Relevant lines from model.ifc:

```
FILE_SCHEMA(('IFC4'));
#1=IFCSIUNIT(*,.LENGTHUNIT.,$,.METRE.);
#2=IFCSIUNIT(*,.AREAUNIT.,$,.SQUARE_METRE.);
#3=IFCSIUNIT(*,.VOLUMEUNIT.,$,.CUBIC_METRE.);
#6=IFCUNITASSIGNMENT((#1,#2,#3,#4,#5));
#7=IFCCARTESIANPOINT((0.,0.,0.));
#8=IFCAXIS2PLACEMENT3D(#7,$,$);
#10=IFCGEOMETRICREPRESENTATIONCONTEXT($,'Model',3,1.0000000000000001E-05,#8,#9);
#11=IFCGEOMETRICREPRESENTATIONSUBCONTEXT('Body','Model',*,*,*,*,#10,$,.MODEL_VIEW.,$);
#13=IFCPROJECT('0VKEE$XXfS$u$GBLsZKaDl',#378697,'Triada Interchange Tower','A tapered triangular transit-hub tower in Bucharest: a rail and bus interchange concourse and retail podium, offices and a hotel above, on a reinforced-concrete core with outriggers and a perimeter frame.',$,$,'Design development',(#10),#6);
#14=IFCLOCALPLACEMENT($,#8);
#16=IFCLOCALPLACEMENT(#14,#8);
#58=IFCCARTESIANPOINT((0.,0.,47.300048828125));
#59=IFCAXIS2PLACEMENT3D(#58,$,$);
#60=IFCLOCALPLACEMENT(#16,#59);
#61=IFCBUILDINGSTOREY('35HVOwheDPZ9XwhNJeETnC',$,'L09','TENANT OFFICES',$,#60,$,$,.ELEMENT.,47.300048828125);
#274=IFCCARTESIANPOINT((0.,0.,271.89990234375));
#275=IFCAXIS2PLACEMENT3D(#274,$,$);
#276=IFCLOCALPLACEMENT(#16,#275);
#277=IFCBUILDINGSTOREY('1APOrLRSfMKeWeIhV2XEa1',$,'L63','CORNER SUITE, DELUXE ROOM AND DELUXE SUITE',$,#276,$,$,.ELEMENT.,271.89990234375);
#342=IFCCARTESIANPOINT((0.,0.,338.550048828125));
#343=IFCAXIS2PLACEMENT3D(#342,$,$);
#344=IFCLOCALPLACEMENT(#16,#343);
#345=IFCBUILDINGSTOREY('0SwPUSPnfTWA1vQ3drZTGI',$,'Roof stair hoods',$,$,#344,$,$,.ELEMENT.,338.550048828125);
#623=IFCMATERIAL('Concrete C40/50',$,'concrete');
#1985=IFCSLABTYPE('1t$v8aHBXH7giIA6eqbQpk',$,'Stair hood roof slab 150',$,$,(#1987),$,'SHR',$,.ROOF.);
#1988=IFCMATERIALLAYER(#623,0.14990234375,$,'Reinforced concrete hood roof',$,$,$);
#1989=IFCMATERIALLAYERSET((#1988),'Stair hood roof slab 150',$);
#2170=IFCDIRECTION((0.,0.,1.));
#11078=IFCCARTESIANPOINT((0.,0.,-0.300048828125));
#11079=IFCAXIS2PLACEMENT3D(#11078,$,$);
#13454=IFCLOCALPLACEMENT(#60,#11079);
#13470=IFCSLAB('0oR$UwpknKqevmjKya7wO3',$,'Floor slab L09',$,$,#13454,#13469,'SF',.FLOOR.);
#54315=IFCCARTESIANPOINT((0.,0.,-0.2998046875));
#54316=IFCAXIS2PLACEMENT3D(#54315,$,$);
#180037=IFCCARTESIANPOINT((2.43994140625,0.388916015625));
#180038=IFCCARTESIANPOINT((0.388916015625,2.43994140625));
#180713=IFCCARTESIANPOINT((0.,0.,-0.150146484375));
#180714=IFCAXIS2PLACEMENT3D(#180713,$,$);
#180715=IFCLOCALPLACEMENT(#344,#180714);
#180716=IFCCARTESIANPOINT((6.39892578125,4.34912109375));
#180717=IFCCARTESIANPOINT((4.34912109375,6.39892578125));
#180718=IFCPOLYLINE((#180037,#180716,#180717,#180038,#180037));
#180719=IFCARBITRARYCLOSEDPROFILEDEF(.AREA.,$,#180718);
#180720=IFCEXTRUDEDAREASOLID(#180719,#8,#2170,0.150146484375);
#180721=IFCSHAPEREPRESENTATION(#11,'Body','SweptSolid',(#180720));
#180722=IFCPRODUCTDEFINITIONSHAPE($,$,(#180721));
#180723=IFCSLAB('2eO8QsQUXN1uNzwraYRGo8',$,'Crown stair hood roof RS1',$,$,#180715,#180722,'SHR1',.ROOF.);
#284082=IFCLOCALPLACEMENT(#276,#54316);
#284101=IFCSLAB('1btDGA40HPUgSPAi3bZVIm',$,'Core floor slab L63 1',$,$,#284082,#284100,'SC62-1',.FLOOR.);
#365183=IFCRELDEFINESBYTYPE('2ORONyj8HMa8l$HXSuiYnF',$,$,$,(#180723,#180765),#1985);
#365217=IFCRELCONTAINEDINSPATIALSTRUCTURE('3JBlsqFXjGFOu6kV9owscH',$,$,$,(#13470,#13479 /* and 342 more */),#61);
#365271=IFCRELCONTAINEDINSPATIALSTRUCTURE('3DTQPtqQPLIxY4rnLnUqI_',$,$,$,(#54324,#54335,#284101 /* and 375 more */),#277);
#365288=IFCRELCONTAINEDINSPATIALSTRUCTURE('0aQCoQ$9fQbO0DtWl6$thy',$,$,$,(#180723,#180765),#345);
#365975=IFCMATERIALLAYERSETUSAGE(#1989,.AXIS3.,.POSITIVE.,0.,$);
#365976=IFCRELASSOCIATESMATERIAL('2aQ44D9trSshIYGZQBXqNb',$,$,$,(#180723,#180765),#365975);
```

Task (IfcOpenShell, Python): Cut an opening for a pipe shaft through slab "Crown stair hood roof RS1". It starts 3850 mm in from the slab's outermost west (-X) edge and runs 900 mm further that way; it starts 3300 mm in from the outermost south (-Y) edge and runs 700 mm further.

```python
import numpy as np
import ifcopenshell
import ifcopenshell.api.feature
import ifcopenshell.api.geometry
import ifcopenshell.api.root
import ifcopenshell.geom
import ifcopenshell.util.placement
import ifcopenshell.util.representation
import ifcopenshell.util.shape
import ifcopenshell.util.unit

model = ifcopenshell.open("model.ifc")
unit_scale = ifcopenshell.util.unit.calculate_unit_scale(model)
settings = ifcopenshell.geom.settings()


def volume(element):
    """Net volume in cubic metres, openings subtracted."""
    shape = ifcopenshell.geom.create_shape(settings, element)
    return ifcopenshell.util.shape.get_volume(shape.geometry)


slab = model.by_guid("2eO8QsQUXN1uNzwraYRGo8")
before = volume(slab)

# Extent in the slab's own axes, in metres. The edges named are its -X and -Y sides.
slab_shape = ifcopenshell.geom.create_shape(settings, slab)
vertices = ifcopenshell.util.shape.get_vertices(slab_shape.geometry)
x_min, y_min, bottom = vertices.min(axis=0)
top = vertices[:, 2].max()

opening = ifcopenshell.api.root.create_entity(model, ifc_class="IfcOpeningElement", name="Pipe shaft opening", predefined_type="OPENING")
context = ifcopenshell.util.representation.get_context(model, "Model", "Body", "MODEL_VIEW")
width, depth = 0.9, 0.7
outline = [(0.0, 0.0), (width, 0.0), (width, depth), (0.0, depth), (0.0, 0.0)]
# Overshoot both faces by 50 mm so the cut is clean.
shape = ifcopenshell.api.geometry.add_slab_representation(
    model, context=context, depth=top - bottom + 0.1, polyline=outline
)
ifcopenshell.api.geometry.assign_representation(model, product=opening, representation=shape)

matrix = ifcopenshell.util.placement.get_local_placement(slab.ObjectPlacement)
matrix[:, 3] = matrix @ np.append(np.array([x_min + 3.85, y_min + 3.3, bottom - 0.05]) / unit_scale, 1.0)
ifcopenshell.api.geometry.edit_object_placement(model, product=opening, matrix=matrix, is_si=False)
ifcopenshell.api.feature.add_feature(model, feature=opening, element=slab)

after = volume(slab)

print(f"slab volume {before:.3f} -> {after:.3f} m3")

model.write("model-out.ifc")
```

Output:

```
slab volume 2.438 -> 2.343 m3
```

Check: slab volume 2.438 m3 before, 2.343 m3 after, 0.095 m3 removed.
